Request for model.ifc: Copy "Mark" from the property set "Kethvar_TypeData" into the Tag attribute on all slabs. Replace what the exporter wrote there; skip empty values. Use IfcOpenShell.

First a look at what the model holds.

```python
import ifcopenshell
import ifcopenshell.util.element

model = ifcopenshell.open("model.ifc")
print(model.schema)
slabs = model.by_type("IfcSlab")
print(len(slabs), "slabs")
for e in slabs[:8]:
    source = ifcopenshell.util.element.get_pset(e, "Kethvar_TypeData", "Mark")
    target = e.Tag
    print(e.id(), repr(source), repr(target), sep=" | ")
```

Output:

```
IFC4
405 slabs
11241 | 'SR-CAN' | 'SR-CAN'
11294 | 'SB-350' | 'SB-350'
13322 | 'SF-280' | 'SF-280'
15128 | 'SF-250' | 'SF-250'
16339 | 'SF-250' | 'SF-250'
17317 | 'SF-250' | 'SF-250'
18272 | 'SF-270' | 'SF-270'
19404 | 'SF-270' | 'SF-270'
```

```python
import ifcopenshell
import ifcopenshell.util.element

model = ifcopenshell.open("model.ifc")

count = 0
for e in model.by_type("IfcSlab"):
    value = ifcopenshell.util.element.get_pset(e, "Kethvar_TypeData", "Mark")
    current = e.Tag
    if not value or not value.strip() or current == value:
        continue
    e.Tag = value
    count += 1

print(count, "slabs updated")

model.write("model-out.ifc")
```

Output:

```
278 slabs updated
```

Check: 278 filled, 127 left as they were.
